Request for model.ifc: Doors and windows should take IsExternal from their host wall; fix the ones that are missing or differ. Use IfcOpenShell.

First a look at what the model holds.

```python
import ifcopenshell
import ifcopenshell.util.element

model = ifcopenshell.open("model.ifc")
print(model.schema)
seen = {}
for e in model.by_type("IfcDoor") + model.by_type("IfcWindow"):
    if not e.FillsVoids:
        continue
    host = e.FillsVoids[0].RelatingOpeningElement.VoidsElements[0].RelatingBuildingElement
    own = ifcopenshell.util.element.get_pset(e, f"Pset_{e.is_a()[3:].removesuffix('StandardCase')}Common", "IsExternal")
    wall = ifcopenshell.util.element.get_pset(host, "Pset_WallCommon", "IsExternal")
    seen[e.is_a(), own, wall] = seen.get((e.is_a(), own, wall), 0) + 1
for (cls, own, wall), count in sorted(seen.items(), key=str):
    print(count, cls, "IsExternal:", own, "| host wall:", wall)
```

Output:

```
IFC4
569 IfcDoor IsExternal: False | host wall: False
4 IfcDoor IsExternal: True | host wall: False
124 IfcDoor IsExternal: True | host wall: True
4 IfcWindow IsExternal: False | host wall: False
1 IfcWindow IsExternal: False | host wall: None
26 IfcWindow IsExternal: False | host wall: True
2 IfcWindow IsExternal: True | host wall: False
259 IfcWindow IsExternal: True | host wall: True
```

```python
import ifcopenshell
import ifcopenshell.api.pset
import ifcopenshell.util.element

model = ifcopenshell.open("model.ifc")

count = 0
for ifc_class, pset_name in (("IfcDoor", "Pset_DoorCommon"), ("IfcWindow", "Pset_WindowCommon")):
    for e in model.by_type(ifc_class):
        if not e.FillsVoids:
            continue
        host = e.FillsVoids[0].RelatingOpeningElement.VoidsElements[0].RelatingBuildingElement
        external = ifcopenshell.util.element.get_pset(host, "Pset_WallCommon", "IsExternal")
        if external is None or ifcopenshell.util.element.get_pset(e, pset_name, "IsExternal") == external:
            continue
        pset = ifcopenshell.api.pset.add_pset(model, product=e, name=pset_name)
        ifcopenshell.api.pset.edit_pset(model, pset=pset, properties={"IsExternal": external})
        count += 1

print(count, "updated")

model.write("model_v2.ifc")
```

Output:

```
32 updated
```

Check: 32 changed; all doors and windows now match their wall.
